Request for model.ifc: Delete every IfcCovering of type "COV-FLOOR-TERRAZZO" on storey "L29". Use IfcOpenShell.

First a look at what the model holds.

```python
import ifcopenshell
import ifcopenshell.util.element

model = ifcopenshell.open("model.ifc")
print(model.schema)
storey = next(s for s in model.by_type("IfcBuildingStorey") if s.Name == "L29")
coverings = [e for e in ifcopenshell.util.element.get_decomposition(storey) if e.is_a("IfcCovering")]
seen = {}
for e in coverings:
    element_type = ifcopenshell.util.element.get_type(e)
    name = element_type.Name if element_type not in (None, e) else None
    seen[name] = seen.get(name, 0) + 1
for name, count in sorted(seen.items(), key=str):
    print(count, "x", name)
```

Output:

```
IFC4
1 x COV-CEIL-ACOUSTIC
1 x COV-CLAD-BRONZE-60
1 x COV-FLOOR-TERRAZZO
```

```python
import ifcopenshell
import ifcopenshell.api.root
import ifcopenshell.util.element

model = ifcopenshell.open("model.ifc")

storey = next(s for s in model.by_type("IfcBuildingStorey") if s.Name == "L29")
coverings = [e for e in ifcopenshell.util.element.get_decomposition(storey) if e.is_a("IfcCovering")]
targets = [e for e in coverings if (t := ifcopenshell.util.element.get_type(e)) not in (None, e) and t.Name == "COV-FLOOR-TERRAZZO"]

for e in targets:
    ifcopenshell.api.root.remove_product(model, product=e)
print(len(targets), "removed")

model.write("model_rev.ifc")
```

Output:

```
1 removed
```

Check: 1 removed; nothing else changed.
